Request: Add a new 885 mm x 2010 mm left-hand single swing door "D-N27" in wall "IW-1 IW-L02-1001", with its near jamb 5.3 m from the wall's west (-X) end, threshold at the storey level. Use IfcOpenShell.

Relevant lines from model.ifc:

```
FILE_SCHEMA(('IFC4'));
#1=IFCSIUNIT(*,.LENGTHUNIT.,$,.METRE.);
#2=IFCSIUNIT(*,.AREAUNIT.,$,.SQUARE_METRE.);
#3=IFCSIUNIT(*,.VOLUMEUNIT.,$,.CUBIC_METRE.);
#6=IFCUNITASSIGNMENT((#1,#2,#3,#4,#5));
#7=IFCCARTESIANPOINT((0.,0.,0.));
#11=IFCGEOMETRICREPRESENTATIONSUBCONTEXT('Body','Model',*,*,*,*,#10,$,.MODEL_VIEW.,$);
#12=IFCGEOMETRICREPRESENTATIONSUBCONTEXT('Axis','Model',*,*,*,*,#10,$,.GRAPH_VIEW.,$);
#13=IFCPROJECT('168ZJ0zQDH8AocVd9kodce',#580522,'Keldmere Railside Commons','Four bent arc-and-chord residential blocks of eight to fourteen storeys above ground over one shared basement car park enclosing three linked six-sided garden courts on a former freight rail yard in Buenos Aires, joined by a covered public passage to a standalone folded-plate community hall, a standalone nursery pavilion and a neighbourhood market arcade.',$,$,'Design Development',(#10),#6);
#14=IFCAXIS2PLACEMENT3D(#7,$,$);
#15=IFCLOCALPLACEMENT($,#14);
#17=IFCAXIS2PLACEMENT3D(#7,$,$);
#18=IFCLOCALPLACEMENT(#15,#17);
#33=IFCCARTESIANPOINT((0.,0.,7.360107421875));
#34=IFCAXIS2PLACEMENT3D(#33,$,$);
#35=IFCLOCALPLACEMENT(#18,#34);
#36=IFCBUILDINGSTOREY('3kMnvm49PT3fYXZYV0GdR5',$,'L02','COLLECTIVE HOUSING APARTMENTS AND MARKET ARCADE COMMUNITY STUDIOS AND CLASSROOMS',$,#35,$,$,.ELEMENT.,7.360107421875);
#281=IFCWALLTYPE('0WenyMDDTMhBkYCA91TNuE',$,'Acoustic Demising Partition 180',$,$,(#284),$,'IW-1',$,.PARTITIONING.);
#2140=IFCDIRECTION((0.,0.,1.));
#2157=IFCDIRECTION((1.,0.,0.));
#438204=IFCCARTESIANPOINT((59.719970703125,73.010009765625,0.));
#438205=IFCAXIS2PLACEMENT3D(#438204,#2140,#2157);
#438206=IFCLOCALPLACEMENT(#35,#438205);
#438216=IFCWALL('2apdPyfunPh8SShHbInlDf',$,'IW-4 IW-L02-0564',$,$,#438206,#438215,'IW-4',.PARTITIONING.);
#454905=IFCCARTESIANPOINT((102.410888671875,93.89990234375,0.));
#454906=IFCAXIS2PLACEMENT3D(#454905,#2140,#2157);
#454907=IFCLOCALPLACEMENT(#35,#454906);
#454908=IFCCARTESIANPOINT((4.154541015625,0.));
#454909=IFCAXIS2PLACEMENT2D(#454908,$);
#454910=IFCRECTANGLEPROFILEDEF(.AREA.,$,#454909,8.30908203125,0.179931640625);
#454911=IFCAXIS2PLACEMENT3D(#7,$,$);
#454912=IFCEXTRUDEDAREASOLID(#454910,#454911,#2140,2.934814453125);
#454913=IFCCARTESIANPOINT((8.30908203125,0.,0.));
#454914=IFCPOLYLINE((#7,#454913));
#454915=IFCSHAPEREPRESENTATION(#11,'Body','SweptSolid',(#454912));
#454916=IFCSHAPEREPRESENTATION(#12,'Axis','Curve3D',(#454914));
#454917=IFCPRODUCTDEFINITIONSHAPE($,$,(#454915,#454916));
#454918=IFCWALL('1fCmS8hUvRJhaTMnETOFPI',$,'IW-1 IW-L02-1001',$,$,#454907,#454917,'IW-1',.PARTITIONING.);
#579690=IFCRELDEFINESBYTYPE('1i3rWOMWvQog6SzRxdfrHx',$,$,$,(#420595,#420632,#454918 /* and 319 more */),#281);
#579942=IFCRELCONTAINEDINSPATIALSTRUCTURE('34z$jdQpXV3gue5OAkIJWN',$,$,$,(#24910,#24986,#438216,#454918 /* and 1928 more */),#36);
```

```python
import numpy as np
import ifcopenshell
import ifcopenshell.api.feature
import ifcopenshell.api.geometry
import ifcopenshell.api.root
import ifcopenshell.api.spatial
import ifcopenshell.geom
import ifcopenshell.util.element
import ifcopenshell.util.placement
import ifcopenshell.util.representation
import ifcopenshell.util.shape
import ifcopenshell.util.unit

model = ifcopenshell.open("model.ifc")
unit_scale = ifcopenshell.util.unit.calculate_unit_scale(model)
settings = ifcopenshell.geom.settings()


def volume(element):
    """Net volume in cubic metres, openings subtracted."""
    shape = ifcopenshell.geom.create_shape(settings, element)
    return ifcopenshell.util.shape.get_volume(shape.geometry)


wall = model.by_guid("1fCmS8hUvRJhaTMnETOFPI")
storey = ifcopenshell.util.element.get_container(wall, ifc_class="IfcBuildingStorey")
context = ifcopenshell.util.representation.get_context(model, "Model", "Body", "MODEL_VIEW")
before = volume(wall)

width, height, from_end, sill = 0.885, 2.01, 5.3, 0.0  # metres

# The wall runs along its own X axis, and the end named is its -X end.
wall_shape = ifcopenshell.geom.create_shape(settings, wall)
x, y, z = ifcopenshell.util.shape.get_vertices(wall_shape.geometry).T
start = x.min() + from_end
face, thickness = float(y.min()), float(y.max() - y.min())
wall_matrix = ifcopenshell.util.placement.get_local_placement(wall.ObjectPlacement)
level = ifcopenshell.util.placement.get_local_placement(storey.ObjectPlacement)[2, 3]


def in_wall(x, y):
    """Placement at x, y metres in the wall's axes, at sill height."""
    matrix = wall_matrix.copy()
    matrix[:, 3] = wall_matrix @ np.array([x / unit_scale, y / unit_scale, 0.0, 1.0])
    matrix[2, 3] = level + sill / unit_scale
    return matrix


# Opening: a box that overshoots both wall faces by 50 mm.
opening = ifcopenshell.api.root.create_entity(model, ifc_class="IfcOpeningElement", predefined_type="OPENING")
box = ifcopenshell.api.geometry.add_wall_representation(
    model, context=context, length=width, height=height, thickness=thickness + 0.1
)
ifcopenshell.api.geometry.assign_representation(model, product=opening, representation=box)
ifcopenshell.api.geometry.edit_object_placement(model, product=opening, matrix=in_wall(start, face - 0.05), is_si=False)
ifcopenshell.api.feature.add_feature(model, feature=opening, element=wall)

door = ifcopenshell.api.root.create_entity(model, ifc_class="IfcDoor", name="D-N27", predefined_type="DOOR")
door.OverallWidth, door.OverallHeight = width / unit_scale, height / unit_scale
door.OperationType = "SINGLE_SWING_LEFT"
body = ifcopenshell.api.geometry.add_door_representation(
    model,
    context=context,
    overall_width=door.OverallWidth,
    overall_height=door.OverallHeight,
    operation_type="SINGLE_SWING_LEFT",
    lining_properties={"LiningDepth": thickness / unit_scale, "ThresholdDepth": thickness / unit_scale},
)
ifcopenshell.api.geometry.assign_representation(model, product=door, representation=body)
ifcopenshell.api.spatial.assign_container(model, products=[door], relating_structure=storey)
ifcopenshell.api.feature.add_filling(model, opening=opening, element=door)

# The lining spans the wall, so the door starts at the wall face.
ifcopenshell.api.geometry.edit_object_placement(model, product=door, matrix=in_wall(start, face), is_si=False)

after = volume(wall)

print(f"wall volume {before:.3f} -> {after:.3f} m3")

model.write("model_updated.ifc")
```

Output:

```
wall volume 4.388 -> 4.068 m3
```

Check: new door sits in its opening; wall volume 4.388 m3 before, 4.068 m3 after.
